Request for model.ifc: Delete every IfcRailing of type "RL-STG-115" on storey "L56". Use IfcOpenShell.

First a look at what the model holds.

```python
import ifcopenshell
import ifcopenshell.util.element

model = ifcopenshell.open("model.ifc")
print(model.schema)
storey = next(s for s in model.by_type("IfcBuildingStorey") if s.Name == "L56")
railings = [e for e in ifcopenshell.util.element.get_decomposition(storey) if e.is_a("IfcRailing")]
seen = {}
for e in railings:
    element_type = ifcopenshell.util.element.get_type(e)
    name = element_type.Name if element_type not in (None, e) else None
    seen[name] = seen.get(name, 0) + 1
for name, count in sorted(seen.items(), key=str):
    print(count, "x", name)
```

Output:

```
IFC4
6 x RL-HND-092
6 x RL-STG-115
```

```python
import ifcopenshell
import ifcopenshell.api.root
import ifcopenshell.util.element

model = ifcopenshell.open("model.ifc")

storey = next(s for s in model.by_type("IfcBuildingStorey") if s.Name == "L56")
railings = [e for e in ifcopenshell.util.element.get_decomposition(storey) if e.is_a("IfcRailing")]
targets = [e for e in railings if (t := ifcopenshell.util.element.get_type(e)) not in (None, e) and t.Name == "RL-STG-115"]

for e in targets:
    ifcopenshell.api.root.remove_product(model, product=e)
print(len(targets), "removed")

model.write("model-out.ifc")
```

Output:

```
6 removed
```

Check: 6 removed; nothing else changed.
